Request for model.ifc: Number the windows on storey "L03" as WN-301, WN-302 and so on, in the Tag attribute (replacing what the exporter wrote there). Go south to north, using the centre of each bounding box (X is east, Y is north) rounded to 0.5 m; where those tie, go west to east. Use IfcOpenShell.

First a look at what the model holds.

```python
import ifcopenshell
import ifcopenshell.util.element
import ifcopenshell.util.placement

model = ifcopenshell.open("model.ifc")
print(model.schema)
storey = next(s for s in model.by_type("IfcBuildingStorey") if s.Name == "L03")
windows = [e for e in ifcopenshell.util.element.get_decomposition(storey) if e.is_a("IfcWindow")]
for e in sorted(windows, key=lambda e: e.id()):
    origin = ifcopenshell.util.placement.get_local_placement(e.ObjectPlacement)[:3, 3]
    print(e.id(), e.Tag, e.Name, origin.round(2) + 0.0, sep=" | ")
```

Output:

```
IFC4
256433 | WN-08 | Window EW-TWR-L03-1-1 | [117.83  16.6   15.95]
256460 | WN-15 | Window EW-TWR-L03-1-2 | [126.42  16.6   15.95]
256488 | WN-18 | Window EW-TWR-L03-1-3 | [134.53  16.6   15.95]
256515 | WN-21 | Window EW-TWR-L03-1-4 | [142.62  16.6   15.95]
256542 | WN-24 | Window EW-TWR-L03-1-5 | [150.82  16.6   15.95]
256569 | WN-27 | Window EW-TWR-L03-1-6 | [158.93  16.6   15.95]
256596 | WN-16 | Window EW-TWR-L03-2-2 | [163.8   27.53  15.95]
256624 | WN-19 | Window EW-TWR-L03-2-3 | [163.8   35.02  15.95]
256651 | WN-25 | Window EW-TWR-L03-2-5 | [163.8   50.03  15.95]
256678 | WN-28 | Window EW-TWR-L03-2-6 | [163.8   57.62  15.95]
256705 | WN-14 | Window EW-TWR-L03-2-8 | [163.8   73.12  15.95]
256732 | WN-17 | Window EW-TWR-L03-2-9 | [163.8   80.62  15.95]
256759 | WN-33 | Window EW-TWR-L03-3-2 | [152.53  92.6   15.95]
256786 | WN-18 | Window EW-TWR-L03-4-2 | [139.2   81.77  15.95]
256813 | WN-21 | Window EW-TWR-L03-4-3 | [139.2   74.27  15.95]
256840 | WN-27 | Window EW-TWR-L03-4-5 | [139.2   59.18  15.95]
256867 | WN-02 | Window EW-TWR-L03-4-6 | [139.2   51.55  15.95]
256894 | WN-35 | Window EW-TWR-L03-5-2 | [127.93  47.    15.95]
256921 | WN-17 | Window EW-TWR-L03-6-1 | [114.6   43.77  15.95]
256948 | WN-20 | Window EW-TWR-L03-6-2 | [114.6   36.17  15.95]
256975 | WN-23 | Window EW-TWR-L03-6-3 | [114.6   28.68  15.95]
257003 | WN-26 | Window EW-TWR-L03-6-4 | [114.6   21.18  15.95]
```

```python
import ifcopenshell
import ifcopenshell.geom
import ifcopenshell.util.element
import ifcopenshell.util.shape

model = ifcopenshell.open("model.ifc")
settings = ifcopenshell.geom.settings()
settings.set("use-world-coords", True)


def centre(element):
    shape = ifcopenshell.geom.create_shape(settings, element)
    return ifcopenshell.util.shape.get_bbox_centroid(shape.geometry)


storey = next(s for s in model.by_type("IfcBuildingStorey") if s.Name == "L03")
windows = [e for e in ifcopenshell.util.element.get_decomposition(storey) if e.is_a("IfcWindow")]

# Insertion points can sit at a corner or the storey origin, so sort by the geometry (in metres).
centres = {e: centre(e) for e in windows}
windows.sort(key=lambda e: (round(centres[e][1] / 0.5), centres[e][0]))

for i, e in enumerate(windows, start=1):
    number = f"WN-3{i:02d}"
    e.Tag = number
    print(e.id(), number)

model.write("model_edited.ifc")
```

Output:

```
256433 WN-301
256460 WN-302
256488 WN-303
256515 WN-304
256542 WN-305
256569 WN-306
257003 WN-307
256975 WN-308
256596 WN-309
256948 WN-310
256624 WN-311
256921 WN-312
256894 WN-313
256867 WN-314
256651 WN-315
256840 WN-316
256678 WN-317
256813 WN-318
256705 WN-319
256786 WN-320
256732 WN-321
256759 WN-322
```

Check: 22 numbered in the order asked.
